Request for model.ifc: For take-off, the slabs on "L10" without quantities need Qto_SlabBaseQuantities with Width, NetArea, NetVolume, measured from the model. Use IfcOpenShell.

First a look at what the model holds.

```python
import ifcopenshell
import ifcopenshell.util.element
import ifcopenshell.util.unit

model = ifcopenshell.open("model.ifc")
print(model.schema)
for unit_type in ("LENGTHUNIT", "AREAUNIT", "VOLUMEUNIT"):
    print(unit_type, ifcopenshell.util.unit.calculate_unit_scale(model, unit_type))
storey = next(s for s in model.by_type("IfcBuildingStorey") if s.Name == "L10")
slabs = [e for e in ifcopenshell.util.element.get_decomposition(storey) if e.is_a("IfcSlab")]
for e in sorted(slabs, key=lambda e: e.id()):
    print(e.id(), e.is_a(), e.Name, list(ifcopenshell.util.element.get_psets(e, qtos_only=True)), sep=" | ")
```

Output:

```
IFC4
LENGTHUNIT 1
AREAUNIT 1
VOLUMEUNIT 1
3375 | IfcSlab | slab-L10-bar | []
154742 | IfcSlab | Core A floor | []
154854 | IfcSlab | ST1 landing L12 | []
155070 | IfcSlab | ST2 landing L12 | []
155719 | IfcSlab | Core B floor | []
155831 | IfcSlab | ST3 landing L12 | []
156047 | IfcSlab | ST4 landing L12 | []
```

```python
import ifcopenshell
import ifcopenshell.api.pset
import ifcopenshell.geom
import ifcopenshell.util.element
import ifcopenshell.util.shape
import ifcopenshell.util.unit

model = ifcopenshell.open("model.ifc")
unit_scale = ifcopenshell.util.unit.calculate_unit_scale(model)
area_scale = ifcopenshell.util.unit.calculate_unit_scale(model, "AREAUNIT")
volume_scale = ifcopenshell.util.unit.calculate_unit_scale(model, "VOLUMEUNIT")
settings = ifcopenshell.geom.settings()

storey = next(s for s in model.by_type("IfcBuildingStorey") if s.Name == "L10")
slabs = [e for e in ifcopenshell.util.element.get_decomposition(storey) if e.is_a("IfcSlab")]

for e in sorted(slabs, key=lambda e: e.id()):
    if ifcopenshell.util.element.get_psets(e, qtos_only=True, should_inherit=False):
        continue
    # Geometry comes back in metres, in the element's own axes.
    shape = ifcopenshell.geom.create_shape(settings, e)
    values = {
        "Width": ifcopenshell.util.shape.get_z(shape.geometry) / unit_scale,
        "NetArea": ifcopenshell.util.shape.get_footprint_area(shape.geometry) / area_scale,
        "NetVolume": ifcopenshell.util.shape.get_volume(shape.geometry) / volume_scale,
    }
    qto = ifcopenshell.api.pset.add_qto(model, product=e, name="Qto_SlabBaseQuantities")
    ifcopenshell.api.pset.edit_qto(model, qto=qto, properties=values)
    print(e.id(), {k: round(v, 3) for k, v in values.items()})

model.write("model_updated.ifc")
```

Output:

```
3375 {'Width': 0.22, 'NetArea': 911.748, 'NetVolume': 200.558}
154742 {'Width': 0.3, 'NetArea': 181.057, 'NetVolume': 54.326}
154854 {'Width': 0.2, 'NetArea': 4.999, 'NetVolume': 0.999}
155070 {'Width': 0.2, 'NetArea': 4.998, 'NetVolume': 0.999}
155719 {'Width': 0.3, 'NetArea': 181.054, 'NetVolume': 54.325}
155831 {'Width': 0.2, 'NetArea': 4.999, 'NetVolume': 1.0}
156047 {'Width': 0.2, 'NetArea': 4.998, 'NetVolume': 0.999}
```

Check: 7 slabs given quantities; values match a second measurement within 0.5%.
